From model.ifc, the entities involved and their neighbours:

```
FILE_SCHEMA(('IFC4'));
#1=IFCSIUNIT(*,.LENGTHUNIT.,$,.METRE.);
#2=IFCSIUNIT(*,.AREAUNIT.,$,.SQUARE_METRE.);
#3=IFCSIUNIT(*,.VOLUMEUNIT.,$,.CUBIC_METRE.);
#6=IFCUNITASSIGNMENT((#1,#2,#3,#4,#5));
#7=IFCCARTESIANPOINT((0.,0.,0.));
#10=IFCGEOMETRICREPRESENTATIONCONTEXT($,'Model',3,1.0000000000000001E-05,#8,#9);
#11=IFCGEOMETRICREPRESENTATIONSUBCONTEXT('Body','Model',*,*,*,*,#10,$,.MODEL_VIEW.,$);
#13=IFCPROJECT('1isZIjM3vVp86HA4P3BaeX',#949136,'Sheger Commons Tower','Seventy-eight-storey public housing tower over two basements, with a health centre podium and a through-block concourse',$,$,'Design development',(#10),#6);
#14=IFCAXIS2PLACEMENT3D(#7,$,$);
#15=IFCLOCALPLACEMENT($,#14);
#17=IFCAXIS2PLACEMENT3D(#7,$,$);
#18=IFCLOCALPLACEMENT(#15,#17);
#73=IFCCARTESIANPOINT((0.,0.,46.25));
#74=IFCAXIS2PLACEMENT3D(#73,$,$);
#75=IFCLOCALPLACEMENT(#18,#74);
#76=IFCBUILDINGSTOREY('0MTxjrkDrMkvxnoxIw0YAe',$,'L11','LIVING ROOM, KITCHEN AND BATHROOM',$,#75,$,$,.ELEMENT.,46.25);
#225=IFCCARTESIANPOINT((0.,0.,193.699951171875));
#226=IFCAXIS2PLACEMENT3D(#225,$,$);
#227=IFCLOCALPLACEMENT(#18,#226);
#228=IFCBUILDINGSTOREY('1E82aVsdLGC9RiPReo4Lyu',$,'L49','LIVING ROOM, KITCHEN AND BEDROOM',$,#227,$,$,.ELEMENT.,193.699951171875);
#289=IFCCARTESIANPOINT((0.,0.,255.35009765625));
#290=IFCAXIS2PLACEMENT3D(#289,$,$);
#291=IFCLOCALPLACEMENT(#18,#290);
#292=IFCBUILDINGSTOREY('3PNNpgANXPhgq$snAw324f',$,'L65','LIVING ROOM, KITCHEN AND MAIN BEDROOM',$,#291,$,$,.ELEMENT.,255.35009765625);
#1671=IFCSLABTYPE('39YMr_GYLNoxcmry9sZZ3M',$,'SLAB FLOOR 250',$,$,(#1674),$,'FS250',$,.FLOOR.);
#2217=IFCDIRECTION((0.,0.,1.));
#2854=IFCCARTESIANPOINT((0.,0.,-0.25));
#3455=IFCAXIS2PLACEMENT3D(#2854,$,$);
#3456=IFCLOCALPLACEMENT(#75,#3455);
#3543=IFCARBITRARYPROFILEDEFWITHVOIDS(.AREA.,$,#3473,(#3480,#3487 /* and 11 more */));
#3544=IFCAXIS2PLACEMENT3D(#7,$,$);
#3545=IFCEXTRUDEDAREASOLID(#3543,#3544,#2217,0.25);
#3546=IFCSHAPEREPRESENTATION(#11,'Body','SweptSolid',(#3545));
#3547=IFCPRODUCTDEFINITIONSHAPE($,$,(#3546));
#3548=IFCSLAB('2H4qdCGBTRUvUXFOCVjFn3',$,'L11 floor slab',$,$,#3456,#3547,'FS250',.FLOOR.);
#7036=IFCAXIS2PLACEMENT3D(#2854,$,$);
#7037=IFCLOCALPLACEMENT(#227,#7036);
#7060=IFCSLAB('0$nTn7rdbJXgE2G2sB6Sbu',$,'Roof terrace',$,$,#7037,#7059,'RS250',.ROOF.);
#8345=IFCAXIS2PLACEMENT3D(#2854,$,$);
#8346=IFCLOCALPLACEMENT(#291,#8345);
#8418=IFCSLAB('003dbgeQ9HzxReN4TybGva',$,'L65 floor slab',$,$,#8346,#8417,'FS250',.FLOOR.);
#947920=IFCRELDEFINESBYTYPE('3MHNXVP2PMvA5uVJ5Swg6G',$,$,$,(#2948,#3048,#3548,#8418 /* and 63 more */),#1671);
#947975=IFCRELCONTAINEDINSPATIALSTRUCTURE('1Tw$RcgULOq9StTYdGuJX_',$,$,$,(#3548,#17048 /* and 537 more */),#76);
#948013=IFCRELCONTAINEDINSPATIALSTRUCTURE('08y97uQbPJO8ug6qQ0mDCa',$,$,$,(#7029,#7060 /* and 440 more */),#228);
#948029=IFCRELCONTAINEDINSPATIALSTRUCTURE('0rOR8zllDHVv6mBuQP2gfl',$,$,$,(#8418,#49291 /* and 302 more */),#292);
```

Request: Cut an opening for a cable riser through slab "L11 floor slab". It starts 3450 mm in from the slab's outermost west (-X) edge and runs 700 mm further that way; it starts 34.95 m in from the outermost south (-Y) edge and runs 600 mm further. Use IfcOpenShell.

```python
import numpy as np
import ifcopenshell
import ifcopenshell.api.feature
import ifcopenshell.api.geometry
import ifcopenshell.api.root
import ifcopenshell.geom
import ifcopenshell.util.placement
import ifcopenshell.util.representation
import ifcopenshell.util.shape
import ifcopenshell.util.unit

model = ifcopenshell.open("model.ifc")
unit_scale = ifcopenshell.util.unit.calculate_unit_scale(model)
settings = ifcopenshell.geom.settings()


def volume(element):
    """Net volume in cubic metres, openings subtracted."""
    shape = ifcopenshell.geom.create_shape(settings, element)
    return ifcopenshell.util.shape.get_volume(shape.geometry)


slab = model.by_guid("2H4qdCGBTRUvUXFOCVjFn3")
before = volume(slab)

# Extent in the slab's own axes, in metres. The edges named are its -X and -Y sides.
slab_shape = ifcopenshell.geom.create_shape(settings, slab)
vertices = ifcopenshell.util.shape.get_vertices(slab_shape.geometry)
x_min, y_min, bottom = vertices.min(axis=0)
top = vertices[:, 2].max()

opening = ifcopenshell.api.root.create_entity(model, ifc_class="IfcOpeningElement", name="Cable riser opening", predefined_type="OPENING")
context = ifcopenshell.util.representation.get_context(model, "Model", "Body", "MODEL_VIEW")
width, depth = 0.7, 0.6
outline = [(0.0, 0.0), (width, 0.0), (width, depth), (0.0, depth), (0.0, 0.0)]
# Overshoot both faces by 50 mm so the cut is clean.
shape = ifcopenshell.api.geometry.add_slab_representation(
    model, context=context, depth=top - bottom + 0.1, polyline=outline
)
ifcopenshell.api.geometry.assign_representation(model, product=opening, representation=shape)

matrix = ifcopenshell.util.placement.get_local_placement(slab.ObjectPlacement)
matrix[:, 3] = matrix @ np.append(np.array([x_min + 3.45, y_min + 34.95, bottom - 0.05]) / unit_scale, 1.0)
ifcopenshell.api.geometry.edit_object_placement(model, product=opening, matrix=matrix, is_si=False)
ifcopenshell.api.feature.add_feature(model, feature=opening, element=slab)

after = volume(slab)

print(f"slab volume {before:.3f} -> {after:.3f} m3")

model.write("model_edited.ifc")
```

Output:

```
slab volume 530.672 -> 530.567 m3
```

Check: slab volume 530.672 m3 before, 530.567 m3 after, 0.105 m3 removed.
